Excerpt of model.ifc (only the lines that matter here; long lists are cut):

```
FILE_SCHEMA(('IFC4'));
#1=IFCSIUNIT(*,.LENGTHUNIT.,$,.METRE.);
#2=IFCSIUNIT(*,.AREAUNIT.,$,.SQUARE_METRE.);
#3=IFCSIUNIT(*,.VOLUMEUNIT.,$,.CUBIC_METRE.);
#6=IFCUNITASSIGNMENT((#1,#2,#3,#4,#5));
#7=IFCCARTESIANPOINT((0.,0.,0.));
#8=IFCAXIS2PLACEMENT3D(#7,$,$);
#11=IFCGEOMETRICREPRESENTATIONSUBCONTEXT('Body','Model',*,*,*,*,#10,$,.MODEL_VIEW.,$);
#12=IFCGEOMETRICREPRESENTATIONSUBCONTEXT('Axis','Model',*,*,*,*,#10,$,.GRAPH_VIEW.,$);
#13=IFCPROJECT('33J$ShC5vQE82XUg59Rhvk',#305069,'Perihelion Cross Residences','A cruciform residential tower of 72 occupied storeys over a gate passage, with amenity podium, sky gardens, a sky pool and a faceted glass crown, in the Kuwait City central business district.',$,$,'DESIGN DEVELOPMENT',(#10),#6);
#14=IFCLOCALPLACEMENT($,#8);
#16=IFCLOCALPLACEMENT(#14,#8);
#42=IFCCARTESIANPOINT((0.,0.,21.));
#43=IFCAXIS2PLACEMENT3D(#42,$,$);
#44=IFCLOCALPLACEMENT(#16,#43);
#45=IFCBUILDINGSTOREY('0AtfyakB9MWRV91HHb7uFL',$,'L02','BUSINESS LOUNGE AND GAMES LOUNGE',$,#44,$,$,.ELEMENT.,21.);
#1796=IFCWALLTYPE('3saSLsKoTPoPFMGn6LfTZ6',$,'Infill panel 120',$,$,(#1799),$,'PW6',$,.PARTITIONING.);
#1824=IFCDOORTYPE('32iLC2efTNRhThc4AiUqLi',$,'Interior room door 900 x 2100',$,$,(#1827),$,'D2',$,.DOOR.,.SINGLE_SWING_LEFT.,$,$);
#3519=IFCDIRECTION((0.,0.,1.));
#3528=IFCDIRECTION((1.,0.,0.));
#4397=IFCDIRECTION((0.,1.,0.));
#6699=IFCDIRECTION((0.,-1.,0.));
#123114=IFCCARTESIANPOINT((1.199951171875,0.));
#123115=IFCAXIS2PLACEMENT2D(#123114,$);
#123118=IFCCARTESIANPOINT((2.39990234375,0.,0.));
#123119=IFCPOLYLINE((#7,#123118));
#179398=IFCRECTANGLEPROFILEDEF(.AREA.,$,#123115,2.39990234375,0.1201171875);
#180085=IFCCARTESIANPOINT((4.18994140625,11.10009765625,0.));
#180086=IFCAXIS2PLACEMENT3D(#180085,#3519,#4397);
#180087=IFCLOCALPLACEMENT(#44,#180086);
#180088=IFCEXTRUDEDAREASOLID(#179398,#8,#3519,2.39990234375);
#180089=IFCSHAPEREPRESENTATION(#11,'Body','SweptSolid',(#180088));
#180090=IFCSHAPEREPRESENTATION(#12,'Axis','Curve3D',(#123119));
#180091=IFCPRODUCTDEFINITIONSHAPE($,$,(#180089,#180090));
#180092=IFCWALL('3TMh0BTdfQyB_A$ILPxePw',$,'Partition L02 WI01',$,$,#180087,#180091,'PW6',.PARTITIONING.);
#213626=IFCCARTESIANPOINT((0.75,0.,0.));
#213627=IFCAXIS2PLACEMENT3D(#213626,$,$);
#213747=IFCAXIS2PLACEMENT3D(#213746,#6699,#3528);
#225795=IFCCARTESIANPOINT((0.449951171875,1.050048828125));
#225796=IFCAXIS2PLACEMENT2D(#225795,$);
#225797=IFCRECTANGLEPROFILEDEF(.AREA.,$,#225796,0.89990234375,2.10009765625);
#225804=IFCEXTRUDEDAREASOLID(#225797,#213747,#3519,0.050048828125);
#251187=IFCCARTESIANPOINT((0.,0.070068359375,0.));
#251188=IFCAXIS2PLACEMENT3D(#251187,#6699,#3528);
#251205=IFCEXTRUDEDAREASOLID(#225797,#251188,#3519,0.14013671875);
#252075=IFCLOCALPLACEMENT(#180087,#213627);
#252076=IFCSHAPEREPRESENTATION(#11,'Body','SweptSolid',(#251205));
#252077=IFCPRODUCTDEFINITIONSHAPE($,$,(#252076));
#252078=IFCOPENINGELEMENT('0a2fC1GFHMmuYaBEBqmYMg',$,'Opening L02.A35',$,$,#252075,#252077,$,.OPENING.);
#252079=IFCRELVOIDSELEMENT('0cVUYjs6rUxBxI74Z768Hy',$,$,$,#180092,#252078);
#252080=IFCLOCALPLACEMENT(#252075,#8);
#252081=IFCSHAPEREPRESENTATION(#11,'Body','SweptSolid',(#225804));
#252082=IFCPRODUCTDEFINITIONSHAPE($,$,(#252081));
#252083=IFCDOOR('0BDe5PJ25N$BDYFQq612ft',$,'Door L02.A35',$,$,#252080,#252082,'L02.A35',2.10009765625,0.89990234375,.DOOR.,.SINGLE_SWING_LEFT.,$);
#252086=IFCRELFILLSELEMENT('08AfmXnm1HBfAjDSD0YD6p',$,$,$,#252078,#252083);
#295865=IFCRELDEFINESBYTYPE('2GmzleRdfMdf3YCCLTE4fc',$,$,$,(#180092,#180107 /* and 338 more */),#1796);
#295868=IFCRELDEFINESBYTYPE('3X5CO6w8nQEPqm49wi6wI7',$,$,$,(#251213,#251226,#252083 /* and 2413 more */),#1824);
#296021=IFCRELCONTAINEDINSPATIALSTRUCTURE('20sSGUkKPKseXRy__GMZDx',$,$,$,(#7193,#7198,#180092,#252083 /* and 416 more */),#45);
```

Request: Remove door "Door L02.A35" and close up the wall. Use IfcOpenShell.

```python
import ifcopenshell
import ifcopenshell.api.feature
import ifcopenshell.api.root
import ifcopenshell.geom
import ifcopenshell.util.shape

model = ifcopenshell.open("model.ifc")
settings = ifcopenshell.geom.settings()


def volume(element):
    """Net volume in cubic metres, openings subtracted."""
    shape = ifcopenshell.geom.create_shape(settings, element)
    return ifcopenshell.util.shape.get_volume(shape.geometry)


door = model.by_guid("0BDe5PJ25N$BDYFQq612ft")
opening = door.FillsVoids[0].RelatingOpeningElement
wall = opening.VoidsElements[0].RelatingBuildingElement
before = volume(wall)

ifcopenshell.api.root.remove_product(model, product=door)
ifcopenshell.api.feature.remove_feature(model, feature=opening)

after = volume(wall)

print(f"wall volume {before:.3f} -> {after:.3f} m3")

model.write("model_v2.ifc")
```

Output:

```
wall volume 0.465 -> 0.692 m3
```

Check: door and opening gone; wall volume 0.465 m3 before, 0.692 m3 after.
